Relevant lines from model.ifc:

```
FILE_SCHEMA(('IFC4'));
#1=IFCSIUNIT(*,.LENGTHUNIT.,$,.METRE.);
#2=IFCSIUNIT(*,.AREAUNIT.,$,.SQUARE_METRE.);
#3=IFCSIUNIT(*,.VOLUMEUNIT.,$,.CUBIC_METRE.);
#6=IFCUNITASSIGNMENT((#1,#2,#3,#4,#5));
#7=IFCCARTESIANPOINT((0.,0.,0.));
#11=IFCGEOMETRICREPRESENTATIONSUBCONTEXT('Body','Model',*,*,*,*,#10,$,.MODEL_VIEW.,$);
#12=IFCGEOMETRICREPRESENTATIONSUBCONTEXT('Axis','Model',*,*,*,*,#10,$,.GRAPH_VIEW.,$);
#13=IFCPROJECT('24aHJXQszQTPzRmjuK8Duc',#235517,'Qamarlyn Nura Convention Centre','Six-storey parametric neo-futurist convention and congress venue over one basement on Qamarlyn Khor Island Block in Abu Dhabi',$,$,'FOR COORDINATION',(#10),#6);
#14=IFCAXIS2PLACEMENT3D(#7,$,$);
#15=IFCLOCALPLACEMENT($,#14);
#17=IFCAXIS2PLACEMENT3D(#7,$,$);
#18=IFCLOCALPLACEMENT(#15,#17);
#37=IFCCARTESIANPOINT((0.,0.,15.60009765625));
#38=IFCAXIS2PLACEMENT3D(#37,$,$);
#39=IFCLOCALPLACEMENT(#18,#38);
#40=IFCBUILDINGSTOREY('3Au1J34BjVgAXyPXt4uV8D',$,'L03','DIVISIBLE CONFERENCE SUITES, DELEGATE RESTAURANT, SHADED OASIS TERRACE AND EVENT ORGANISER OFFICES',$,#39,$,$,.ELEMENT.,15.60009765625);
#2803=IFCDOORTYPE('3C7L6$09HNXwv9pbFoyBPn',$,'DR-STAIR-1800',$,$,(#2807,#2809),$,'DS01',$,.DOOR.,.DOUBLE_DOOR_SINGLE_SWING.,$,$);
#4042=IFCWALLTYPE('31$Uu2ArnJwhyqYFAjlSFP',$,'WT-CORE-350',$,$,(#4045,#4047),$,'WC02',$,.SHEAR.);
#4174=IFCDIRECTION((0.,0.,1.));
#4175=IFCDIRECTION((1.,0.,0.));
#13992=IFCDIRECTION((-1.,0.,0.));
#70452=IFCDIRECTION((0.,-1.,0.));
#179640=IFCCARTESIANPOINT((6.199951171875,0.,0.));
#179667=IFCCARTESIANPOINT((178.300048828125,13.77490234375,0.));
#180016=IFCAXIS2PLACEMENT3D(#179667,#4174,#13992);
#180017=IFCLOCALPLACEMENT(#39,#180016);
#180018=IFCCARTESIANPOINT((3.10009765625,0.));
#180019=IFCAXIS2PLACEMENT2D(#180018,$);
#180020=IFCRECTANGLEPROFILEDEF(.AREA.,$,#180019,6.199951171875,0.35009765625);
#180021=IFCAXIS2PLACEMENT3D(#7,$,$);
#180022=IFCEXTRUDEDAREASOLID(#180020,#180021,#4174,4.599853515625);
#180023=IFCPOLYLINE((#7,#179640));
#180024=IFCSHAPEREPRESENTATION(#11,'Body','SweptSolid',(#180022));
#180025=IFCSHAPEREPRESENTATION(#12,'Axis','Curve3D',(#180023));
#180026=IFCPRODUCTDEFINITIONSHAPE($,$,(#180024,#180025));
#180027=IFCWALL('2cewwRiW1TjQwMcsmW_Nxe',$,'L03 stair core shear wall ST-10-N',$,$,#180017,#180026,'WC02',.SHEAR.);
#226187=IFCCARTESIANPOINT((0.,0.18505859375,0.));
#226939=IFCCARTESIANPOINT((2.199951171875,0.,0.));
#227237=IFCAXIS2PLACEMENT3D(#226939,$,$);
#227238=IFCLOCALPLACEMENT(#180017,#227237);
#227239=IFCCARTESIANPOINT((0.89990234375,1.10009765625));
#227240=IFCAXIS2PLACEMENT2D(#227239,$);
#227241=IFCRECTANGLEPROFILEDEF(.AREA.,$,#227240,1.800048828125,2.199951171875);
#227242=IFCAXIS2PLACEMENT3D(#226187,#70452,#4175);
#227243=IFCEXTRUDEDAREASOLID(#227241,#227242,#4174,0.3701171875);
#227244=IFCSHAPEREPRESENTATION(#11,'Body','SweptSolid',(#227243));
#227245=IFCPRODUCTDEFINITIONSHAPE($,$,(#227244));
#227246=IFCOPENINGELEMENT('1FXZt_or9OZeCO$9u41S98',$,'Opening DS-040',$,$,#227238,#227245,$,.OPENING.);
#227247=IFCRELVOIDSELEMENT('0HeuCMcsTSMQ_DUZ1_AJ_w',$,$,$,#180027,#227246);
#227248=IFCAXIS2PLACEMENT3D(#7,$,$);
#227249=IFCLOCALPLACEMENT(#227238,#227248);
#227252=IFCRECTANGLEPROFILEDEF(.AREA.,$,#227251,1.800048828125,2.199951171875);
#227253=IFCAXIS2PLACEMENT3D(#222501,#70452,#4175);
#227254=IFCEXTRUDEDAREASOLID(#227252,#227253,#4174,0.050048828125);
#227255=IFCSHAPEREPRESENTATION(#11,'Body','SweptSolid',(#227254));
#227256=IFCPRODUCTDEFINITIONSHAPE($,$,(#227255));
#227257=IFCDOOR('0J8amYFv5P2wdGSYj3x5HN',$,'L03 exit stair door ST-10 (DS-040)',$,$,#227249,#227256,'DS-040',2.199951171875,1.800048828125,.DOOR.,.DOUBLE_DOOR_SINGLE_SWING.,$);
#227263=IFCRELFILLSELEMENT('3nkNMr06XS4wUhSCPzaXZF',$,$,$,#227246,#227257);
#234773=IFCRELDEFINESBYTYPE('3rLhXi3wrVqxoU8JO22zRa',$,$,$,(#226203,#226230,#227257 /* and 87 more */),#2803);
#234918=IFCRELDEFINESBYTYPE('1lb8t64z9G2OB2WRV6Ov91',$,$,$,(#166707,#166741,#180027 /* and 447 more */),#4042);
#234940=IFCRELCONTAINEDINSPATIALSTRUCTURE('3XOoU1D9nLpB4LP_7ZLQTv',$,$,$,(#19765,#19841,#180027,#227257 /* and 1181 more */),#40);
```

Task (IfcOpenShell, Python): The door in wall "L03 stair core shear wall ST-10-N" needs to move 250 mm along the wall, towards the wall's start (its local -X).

```python
import ifcopenshell
import ifcopenshell.api.geometry
import ifcopenshell.util.placement
import ifcopenshell.util.unit

model = ifcopenshell.open("model.ifc")
unit_scale = ifcopenshell.util.unit.calculate_unit_scale(model)

door = model.by_id(227257)
opening = door.FillsVoids[0].RelatingOpeningElement
wall = opening.VoidsElements[0].RelatingBuildingElement

wall_matrix = ifcopenshell.util.placement.get_local_placement(wall.ObjectPlacement)
shift = wall_matrix[:3, 0] * -0.25 / unit_scale
before = ifcopenshell.util.placement.get_local_placement(door.ObjectPlacement)[:3, 3].copy()

# The door is placed relative to its opening, so it follows when the opening moves.
matrix = ifcopenshell.util.placement.get_local_placement(opening.ObjectPlacement)
matrix[:3, 3] += shift
ifcopenshell.api.geometry.edit_object_placement(
    model, product=opening, matrix=matrix, is_si=False, should_transform_children=True
)

after = ifcopenshell.util.placement.get_local_placement(door.ObjectPlacement)[:3, 3]
print("door moved by", (after - before).round(3) + 0.0)

model.write("model-out.ifc")
```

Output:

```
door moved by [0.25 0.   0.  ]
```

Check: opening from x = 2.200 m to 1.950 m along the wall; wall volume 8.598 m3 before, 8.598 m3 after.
